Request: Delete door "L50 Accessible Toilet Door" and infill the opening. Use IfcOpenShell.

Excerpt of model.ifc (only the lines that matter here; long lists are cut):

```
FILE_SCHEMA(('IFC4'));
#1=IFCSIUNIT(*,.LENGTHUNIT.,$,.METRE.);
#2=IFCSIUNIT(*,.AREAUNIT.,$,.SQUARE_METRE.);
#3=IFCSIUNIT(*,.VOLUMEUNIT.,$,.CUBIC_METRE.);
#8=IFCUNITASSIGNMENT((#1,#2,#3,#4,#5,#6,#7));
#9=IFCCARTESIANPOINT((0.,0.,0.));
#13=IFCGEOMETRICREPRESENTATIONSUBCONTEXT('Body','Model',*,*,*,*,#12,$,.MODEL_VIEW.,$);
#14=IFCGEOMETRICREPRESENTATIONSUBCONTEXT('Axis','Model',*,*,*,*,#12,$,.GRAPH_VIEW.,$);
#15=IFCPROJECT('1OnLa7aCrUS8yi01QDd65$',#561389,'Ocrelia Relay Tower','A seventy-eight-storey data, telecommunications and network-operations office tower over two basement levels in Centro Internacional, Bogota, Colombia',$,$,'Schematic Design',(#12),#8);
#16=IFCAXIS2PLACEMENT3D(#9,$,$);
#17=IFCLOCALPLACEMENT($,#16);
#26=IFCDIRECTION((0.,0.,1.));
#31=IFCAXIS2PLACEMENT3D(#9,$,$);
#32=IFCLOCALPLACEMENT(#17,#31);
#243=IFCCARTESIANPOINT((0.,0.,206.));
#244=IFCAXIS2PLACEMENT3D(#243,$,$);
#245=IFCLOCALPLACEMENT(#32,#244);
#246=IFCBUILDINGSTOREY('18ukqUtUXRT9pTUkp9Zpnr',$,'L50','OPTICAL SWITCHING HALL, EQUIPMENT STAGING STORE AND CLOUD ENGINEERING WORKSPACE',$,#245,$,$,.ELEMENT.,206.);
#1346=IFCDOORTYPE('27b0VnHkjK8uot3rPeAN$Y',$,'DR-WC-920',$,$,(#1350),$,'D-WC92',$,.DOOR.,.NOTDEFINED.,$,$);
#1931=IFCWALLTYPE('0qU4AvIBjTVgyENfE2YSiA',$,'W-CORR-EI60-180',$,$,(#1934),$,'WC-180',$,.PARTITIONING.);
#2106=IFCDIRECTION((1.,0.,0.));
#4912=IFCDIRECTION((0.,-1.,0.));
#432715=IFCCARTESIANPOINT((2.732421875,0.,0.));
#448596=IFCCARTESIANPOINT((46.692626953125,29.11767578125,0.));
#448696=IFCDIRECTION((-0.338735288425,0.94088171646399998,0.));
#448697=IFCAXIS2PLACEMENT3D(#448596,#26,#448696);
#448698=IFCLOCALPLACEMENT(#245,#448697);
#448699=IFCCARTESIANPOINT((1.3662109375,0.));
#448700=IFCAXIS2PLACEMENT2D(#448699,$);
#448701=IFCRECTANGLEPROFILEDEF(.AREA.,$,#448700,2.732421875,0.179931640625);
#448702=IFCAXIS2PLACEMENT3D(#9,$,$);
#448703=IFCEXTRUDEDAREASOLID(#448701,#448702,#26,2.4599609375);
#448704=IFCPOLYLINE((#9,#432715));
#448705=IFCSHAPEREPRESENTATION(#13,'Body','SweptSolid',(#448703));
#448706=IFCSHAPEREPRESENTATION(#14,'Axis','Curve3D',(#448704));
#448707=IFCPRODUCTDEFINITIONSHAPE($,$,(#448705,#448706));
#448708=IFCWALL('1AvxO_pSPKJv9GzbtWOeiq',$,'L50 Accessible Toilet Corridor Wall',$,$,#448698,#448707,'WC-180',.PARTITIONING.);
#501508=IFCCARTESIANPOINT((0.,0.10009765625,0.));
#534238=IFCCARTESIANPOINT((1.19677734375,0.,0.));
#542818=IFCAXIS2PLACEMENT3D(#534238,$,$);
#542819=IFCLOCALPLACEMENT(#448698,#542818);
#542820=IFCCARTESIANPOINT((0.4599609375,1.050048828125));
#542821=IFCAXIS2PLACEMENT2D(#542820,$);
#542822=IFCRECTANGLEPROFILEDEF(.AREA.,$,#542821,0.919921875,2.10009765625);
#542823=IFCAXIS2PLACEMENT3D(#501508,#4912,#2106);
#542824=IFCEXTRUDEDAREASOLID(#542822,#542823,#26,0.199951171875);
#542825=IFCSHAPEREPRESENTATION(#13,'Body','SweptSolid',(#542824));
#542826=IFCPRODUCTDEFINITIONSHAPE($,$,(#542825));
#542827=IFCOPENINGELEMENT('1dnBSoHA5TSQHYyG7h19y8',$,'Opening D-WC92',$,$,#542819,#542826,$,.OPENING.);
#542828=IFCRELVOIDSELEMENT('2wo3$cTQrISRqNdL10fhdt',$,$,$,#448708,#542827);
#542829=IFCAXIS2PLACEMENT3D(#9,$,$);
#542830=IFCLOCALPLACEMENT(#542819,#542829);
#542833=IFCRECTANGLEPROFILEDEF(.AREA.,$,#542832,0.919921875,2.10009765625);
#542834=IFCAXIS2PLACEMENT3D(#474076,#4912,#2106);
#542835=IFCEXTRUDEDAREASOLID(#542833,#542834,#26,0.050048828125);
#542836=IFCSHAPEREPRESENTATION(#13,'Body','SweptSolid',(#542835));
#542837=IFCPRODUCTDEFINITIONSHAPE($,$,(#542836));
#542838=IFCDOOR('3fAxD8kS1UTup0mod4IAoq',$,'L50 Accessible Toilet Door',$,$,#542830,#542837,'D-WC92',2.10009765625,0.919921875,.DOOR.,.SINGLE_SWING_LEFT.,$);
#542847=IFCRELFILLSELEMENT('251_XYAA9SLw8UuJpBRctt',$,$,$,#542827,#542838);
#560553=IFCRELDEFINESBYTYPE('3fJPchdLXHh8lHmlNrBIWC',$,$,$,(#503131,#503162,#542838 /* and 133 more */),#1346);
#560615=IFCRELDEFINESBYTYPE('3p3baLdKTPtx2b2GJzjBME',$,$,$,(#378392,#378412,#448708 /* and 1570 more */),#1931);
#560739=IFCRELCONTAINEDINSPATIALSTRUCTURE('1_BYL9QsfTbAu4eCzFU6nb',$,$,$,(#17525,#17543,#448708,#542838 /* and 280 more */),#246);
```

```python
import ifcopenshell
import ifcopenshell.api.feature
import ifcopenshell.api.root
import ifcopenshell.geom
import ifcopenshell.util.shape

model = ifcopenshell.open("model.ifc")
settings = ifcopenshell.geom.settings()


def volume(element):
    """Net volume in cubic metres, openings subtracted."""
    shape = ifcopenshell.geom.create_shape(settings, element)
    return ifcopenshell.util.shape.get_volume(shape.geometry)


door = model.by_guid("3fAxD8kS1UTup0mod4IAoq")
opening = door.FillsVoids[0].RelatingOpeningElement
wall = opening.VoidsElements[0].RelatingBuildingElement
before = volume(wall)

ifcopenshell.api.root.remove_product(model, product=door)
ifcopenshell.api.feature.remove_feature(model, feature=opening)

after = volume(wall)

print(f"wall volume {before:.3f} -> {after:.3f} m3")

model.write("model_v2.ifc")
```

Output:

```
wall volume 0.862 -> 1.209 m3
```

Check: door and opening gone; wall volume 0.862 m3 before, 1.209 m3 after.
